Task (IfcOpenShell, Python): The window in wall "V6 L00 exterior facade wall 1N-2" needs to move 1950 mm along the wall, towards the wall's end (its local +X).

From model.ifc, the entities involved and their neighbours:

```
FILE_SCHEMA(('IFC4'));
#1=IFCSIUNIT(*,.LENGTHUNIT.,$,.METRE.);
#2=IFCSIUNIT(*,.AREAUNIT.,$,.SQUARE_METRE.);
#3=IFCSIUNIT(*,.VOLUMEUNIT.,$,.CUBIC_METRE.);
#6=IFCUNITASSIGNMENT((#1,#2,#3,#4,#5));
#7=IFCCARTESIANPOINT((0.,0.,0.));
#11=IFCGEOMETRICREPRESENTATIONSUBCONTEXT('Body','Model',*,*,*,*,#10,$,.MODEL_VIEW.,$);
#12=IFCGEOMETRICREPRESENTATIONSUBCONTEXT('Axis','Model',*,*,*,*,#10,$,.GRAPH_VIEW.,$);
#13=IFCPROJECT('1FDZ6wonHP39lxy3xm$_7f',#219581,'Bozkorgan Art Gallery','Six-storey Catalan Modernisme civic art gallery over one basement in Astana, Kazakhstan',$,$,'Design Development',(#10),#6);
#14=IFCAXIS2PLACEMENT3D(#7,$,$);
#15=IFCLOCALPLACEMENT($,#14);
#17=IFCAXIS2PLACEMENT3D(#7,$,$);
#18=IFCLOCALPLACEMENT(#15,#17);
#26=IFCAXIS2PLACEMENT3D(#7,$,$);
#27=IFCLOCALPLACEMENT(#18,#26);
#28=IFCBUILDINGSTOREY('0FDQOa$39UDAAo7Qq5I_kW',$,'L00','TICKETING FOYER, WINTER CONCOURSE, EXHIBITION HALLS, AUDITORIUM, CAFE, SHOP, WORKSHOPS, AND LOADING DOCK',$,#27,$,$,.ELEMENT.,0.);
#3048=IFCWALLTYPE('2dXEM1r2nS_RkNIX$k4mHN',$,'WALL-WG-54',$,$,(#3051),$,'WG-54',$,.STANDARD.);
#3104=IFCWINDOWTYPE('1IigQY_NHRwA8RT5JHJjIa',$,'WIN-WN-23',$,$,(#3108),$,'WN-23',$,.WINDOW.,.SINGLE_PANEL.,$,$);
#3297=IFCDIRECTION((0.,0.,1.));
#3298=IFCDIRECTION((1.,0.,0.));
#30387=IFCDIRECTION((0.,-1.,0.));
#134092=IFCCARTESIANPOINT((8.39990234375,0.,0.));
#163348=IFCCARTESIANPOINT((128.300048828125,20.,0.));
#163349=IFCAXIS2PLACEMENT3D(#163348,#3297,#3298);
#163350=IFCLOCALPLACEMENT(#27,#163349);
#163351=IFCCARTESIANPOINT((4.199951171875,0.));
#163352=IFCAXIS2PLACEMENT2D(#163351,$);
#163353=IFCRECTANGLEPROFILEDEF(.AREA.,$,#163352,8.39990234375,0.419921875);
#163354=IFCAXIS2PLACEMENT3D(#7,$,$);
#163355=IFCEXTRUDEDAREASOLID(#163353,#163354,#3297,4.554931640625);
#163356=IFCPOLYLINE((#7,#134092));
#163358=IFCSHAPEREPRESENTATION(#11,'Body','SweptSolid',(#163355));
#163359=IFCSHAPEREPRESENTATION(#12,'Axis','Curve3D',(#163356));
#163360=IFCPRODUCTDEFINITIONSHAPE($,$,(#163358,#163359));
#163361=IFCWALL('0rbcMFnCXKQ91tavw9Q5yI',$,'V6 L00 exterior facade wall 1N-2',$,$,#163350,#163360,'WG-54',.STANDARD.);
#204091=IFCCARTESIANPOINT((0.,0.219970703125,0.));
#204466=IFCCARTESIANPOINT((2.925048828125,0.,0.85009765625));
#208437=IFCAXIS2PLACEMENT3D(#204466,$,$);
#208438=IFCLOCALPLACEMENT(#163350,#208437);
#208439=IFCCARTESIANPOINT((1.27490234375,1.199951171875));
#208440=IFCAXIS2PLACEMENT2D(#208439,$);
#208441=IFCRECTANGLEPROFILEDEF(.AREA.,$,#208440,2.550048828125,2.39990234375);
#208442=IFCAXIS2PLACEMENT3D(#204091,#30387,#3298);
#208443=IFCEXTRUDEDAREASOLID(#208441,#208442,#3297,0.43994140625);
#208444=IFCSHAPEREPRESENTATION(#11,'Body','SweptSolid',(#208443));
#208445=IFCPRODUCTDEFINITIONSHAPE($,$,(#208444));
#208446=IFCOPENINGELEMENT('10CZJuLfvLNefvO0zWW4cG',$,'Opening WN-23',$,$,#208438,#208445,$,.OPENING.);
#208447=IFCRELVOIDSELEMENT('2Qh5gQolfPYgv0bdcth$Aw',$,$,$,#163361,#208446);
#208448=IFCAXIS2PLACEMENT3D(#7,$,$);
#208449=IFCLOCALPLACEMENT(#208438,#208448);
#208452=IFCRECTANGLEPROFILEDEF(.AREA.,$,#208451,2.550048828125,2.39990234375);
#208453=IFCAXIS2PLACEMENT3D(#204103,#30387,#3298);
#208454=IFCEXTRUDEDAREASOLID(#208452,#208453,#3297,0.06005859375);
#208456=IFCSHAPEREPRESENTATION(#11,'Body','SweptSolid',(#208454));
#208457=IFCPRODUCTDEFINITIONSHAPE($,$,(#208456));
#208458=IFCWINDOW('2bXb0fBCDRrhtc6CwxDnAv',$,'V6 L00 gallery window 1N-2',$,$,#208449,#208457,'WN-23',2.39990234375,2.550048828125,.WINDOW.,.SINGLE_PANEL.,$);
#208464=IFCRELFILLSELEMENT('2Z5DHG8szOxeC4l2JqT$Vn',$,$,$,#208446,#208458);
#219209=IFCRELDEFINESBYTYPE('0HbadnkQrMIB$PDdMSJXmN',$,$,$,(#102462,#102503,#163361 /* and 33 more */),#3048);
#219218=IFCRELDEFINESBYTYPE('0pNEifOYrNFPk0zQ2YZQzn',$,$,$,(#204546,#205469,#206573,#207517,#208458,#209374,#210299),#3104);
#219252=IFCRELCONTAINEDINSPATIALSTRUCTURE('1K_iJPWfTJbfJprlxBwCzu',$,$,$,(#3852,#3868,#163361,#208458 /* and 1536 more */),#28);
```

```python
import ifcopenshell
import ifcopenshell.api.geometry
import ifcopenshell.util.placement

model = ifcopenshell.open("model.ifc")

window = model.by_id(208458)
opening = window.FillsVoids[0].RelatingOpeningElement
wall = opening.VoidsElements[0].RelatingBuildingElement

wall_matrix = ifcopenshell.util.placement.get_local_placement(wall.ObjectPlacement)
shift = wall_matrix[:3, 0] * 1.95
before = ifcopenshell.util.placement.get_local_placement(window.ObjectPlacement)[:3, 3].copy()

# The window is placed relative to its opening, so it follows when the opening moves.
matrix = ifcopenshell.util.placement.get_local_placement(opening.ObjectPlacement)
matrix[:3, 3] += shift
ifcopenshell.api.geometry.edit_object_placement(
    model, product=opening, matrix=matrix, is_si=False, should_transform_children=True
)

after = ifcopenshell.util.placement.get_local_placement(window.ObjectPlacement)[:3, 3]
print("window moved by", (after - before).round(3) + 0.0)

model.write("model_v2.ifc")
```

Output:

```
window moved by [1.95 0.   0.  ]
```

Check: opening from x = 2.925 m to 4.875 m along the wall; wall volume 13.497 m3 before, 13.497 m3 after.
